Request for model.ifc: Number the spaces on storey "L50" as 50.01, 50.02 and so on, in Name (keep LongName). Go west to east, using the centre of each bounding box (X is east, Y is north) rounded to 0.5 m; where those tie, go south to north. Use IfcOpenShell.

First a look at what the model holds.

```python
import ifcopenshell
import ifcopenshell.util.element
import ifcopenshell.util.placement

model = ifcopenshell.open("model.ifc")
print(model.schema)
storey = next(s for s in model.by_type("IfcBuildingStorey") if s.Name == "L50")
spaces = [e for e in ifcopenshell.util.element.get_decomposition(storey) if e.is_a("IfcSpace")]
for e in sorted(spaces, key=lambda e: e.id()):
    origin = ifcopenshell.util.placement.get_local_placement(e.ObjectPlacement)[:3, 3]
    print(e.id(), e.Name, e.LongName, origin.round(2) + 0.0, sep=" | ")
```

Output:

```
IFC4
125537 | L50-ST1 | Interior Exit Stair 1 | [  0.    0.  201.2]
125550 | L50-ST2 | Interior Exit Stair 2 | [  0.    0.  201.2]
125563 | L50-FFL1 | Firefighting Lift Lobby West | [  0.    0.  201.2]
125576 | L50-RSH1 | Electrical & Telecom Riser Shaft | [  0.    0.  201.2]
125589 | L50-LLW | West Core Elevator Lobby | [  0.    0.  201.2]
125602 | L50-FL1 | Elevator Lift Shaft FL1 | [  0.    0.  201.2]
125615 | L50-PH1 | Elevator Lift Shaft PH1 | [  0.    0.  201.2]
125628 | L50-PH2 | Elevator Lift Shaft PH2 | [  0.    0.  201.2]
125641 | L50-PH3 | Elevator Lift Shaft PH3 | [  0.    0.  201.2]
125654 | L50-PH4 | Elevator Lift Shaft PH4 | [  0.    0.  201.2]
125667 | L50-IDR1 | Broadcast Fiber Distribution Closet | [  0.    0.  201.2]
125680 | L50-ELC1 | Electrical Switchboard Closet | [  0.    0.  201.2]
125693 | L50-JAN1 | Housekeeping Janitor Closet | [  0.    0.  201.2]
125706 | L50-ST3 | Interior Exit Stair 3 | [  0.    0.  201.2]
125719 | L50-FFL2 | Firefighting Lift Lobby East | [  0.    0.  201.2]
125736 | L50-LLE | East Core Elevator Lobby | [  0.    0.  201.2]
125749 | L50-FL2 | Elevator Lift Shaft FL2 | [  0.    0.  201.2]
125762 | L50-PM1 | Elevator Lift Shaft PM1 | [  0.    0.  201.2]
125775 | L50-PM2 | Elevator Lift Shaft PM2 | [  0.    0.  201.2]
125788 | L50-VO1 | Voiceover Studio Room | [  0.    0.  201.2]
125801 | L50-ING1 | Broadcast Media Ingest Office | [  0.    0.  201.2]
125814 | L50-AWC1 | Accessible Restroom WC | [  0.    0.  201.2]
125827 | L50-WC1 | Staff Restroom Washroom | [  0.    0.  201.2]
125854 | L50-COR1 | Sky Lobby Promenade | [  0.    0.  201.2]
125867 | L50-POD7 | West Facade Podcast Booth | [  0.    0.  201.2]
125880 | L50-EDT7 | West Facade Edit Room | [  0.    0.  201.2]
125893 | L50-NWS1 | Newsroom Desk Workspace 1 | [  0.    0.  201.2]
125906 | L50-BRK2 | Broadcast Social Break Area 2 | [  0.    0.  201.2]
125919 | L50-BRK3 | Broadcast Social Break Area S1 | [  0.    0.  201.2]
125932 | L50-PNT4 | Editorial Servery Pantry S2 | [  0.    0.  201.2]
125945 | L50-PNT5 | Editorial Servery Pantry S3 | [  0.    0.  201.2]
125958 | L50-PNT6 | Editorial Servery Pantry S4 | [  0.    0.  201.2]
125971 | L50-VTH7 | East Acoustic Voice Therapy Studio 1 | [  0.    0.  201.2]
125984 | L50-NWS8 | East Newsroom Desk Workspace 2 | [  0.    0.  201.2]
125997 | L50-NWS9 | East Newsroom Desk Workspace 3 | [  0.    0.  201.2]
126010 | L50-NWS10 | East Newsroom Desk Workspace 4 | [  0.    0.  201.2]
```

```python
import ifcopenshell
import ifcopenshell.geom
import ifcopenshell.util.element
import ifcopenshell.util.shape

model = ifcopenshell.open("model.ifc")
settings = ifcopenshell.geom.settings()
settings.set("use-world-coords", True)


def centre(element):
    shape = ifcopenshell.geom.create_shape(settings, element)
    return ifcopenshell.util.shape.get_bbox_centroid(shape.geometry)


storey = next(s for s in model.by_type("IfcBuildingStorey") if s.Name == "L50")
spaces = [e for e in ifcopenshell.util.element.get_decomposition(storey) if e.is_a("IfcSpace")]

# Insertion points can sit at a corner or the storey origin, so sort by the geometry (in metres).
centres = {e: centre(e) for e in spaces}
spaces.sort(key=lambda e: (round(centres[e][0] / 0.5), centres[e][1]))

for i, e in enumerate(spaces, start=1):
    number = f"50.{i:02d}"
    e.Name = number
    print(e.id(), number)

model.write("model_v2.ifc")
```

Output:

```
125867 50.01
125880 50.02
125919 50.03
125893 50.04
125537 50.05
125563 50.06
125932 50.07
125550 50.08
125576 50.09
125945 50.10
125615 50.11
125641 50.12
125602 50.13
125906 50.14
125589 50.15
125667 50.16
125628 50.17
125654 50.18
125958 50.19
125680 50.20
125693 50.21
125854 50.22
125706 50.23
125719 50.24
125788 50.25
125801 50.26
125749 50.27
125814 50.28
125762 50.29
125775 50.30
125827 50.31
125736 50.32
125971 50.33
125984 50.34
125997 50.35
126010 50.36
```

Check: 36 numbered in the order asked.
